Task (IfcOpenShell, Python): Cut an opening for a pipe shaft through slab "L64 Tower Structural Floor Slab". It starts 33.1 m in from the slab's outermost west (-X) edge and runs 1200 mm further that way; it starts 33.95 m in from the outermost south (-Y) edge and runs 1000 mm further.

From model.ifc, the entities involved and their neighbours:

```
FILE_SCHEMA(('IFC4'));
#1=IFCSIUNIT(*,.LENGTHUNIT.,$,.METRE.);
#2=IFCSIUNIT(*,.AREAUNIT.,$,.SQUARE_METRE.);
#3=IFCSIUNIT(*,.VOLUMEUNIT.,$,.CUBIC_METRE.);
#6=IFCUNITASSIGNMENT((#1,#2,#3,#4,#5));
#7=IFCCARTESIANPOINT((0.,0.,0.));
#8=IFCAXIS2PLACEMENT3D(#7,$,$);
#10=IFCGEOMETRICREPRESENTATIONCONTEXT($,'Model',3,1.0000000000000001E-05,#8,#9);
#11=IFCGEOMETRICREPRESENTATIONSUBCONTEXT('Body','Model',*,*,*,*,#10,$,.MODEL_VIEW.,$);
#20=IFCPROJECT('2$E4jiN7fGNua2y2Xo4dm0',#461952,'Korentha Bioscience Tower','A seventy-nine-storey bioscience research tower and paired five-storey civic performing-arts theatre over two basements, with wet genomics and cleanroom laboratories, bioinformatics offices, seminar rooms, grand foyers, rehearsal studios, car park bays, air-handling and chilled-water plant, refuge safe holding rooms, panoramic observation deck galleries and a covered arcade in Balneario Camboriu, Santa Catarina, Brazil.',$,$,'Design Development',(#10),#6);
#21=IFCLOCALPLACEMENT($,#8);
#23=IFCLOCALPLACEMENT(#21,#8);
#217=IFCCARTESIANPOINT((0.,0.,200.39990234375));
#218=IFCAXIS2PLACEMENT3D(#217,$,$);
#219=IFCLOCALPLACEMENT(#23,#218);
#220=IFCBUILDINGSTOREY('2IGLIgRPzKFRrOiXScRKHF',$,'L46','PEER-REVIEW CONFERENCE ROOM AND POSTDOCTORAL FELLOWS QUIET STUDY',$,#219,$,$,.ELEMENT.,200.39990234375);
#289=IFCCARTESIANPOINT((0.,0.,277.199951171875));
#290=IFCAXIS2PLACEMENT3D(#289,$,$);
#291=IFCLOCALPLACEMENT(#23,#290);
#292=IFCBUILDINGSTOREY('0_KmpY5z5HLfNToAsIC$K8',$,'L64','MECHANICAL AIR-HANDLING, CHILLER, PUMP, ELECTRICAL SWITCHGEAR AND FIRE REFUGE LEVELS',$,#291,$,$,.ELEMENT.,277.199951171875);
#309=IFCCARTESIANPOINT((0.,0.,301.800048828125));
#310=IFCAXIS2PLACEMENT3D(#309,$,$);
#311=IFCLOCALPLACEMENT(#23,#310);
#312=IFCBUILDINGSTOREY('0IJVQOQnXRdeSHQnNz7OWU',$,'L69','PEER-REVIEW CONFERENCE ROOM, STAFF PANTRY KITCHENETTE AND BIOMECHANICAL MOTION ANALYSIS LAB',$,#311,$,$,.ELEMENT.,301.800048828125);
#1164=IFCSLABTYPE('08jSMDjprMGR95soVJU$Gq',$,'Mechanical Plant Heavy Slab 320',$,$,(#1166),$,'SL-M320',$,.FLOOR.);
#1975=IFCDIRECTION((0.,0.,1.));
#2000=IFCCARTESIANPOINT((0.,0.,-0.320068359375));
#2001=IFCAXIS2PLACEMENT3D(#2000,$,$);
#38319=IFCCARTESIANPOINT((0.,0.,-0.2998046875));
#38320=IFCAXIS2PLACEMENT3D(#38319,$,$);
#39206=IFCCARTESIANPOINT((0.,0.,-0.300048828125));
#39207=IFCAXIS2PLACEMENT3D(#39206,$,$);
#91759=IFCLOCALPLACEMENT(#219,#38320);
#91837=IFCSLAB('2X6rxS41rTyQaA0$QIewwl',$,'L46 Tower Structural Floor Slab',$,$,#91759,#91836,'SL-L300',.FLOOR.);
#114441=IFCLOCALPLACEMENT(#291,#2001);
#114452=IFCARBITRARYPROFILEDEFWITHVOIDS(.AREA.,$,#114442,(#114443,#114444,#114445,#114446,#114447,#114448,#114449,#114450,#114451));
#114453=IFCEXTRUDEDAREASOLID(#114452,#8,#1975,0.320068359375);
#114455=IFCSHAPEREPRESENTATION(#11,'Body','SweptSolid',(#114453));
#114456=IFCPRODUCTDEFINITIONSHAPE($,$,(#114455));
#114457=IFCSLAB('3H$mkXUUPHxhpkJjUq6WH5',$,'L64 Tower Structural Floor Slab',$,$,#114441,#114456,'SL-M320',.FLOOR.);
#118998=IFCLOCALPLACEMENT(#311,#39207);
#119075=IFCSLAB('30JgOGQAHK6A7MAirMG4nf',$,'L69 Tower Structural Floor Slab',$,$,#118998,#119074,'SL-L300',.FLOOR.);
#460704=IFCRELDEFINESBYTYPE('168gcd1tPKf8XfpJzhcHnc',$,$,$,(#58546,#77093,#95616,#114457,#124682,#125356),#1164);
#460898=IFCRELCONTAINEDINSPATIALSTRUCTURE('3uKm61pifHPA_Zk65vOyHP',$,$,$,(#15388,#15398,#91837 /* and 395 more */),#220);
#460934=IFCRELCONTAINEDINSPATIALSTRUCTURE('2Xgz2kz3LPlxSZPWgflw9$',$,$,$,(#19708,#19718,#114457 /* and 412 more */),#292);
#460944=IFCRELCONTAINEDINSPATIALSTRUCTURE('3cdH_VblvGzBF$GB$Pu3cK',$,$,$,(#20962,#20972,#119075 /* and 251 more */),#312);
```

```python
import numpy as np
import ifcopenshell
import ifcopenshell.api.feature
import ifcopenshell.api.geometry
import ifcopenshell.api.root
import ifcopenshell.geom
import ifcopenshell.util.placement
import ifcopenshell.util.representation
import ifcopenshell.util.shape
import ifcopenshell.util.unit

model = ifcopenshell.open("model.ifc")
unit_scale = ifcopenshell.util.unit.calculate_unit_scale(model)
settings = ifcopenshell.geom.settings()


def volume(element):
    """Net volume in cubic metres, openings subtracted."""
    shape = ifcopenshell.geom.create_shape(settings, element)
    return ifcopenshell.util.shape.get_volume(shape.geometry)


slab = model.by_id(114457)
before = volume(slab)

# Extent in the slab's own axes, in metres. The edges named are its -X and -Y sides.
slab_shape = ifcopenshell.geom.create_shape(settings, slab)
vertices = ifcopenshell.util.shape.get_vertices(slab_shape.geometry)
x_min, y_min, bottom = vertices.min(axis=0)
top = vertices[:, 2].max()

opening = ifcopenshell.api.root.create_entity(model, ifc_class="IfcOpeningElement", name="Pipe shaft opening", predefined_type="OPENING")
context = ifcopenshell.util.representation.get_context(model, "Model", "Body", "MODEL_VIEW")
width, depth = 1.2, 1
outline = [(0.0, 0.0), (width, 0.0), (width, depth), (0.0, depth), (0.0, 0.0)]
# Overshoot both faces by 50 mm so the cut is clean.
shape = ifcopenshell.api.geometry.add_slab_representation(
    model, context=context, depth=top - bottom + 0.1, polyline=outline
)
ifcopenshell.api.geometry.assign_representation(model, product=opening, representation=shape)

matrix = ifcopenshell.util.placement.get_local_placement(slab.ObjectPlacement)
matrix[:, 3] = matrix @ np.append(np.array([x_min + 33.1, y_min + 33.95, bottom - 0.05]) / unit_scale, 1.0)
ifcopenshell.api.geometry.edit_object_placement(model, product=opening, matrix=matrix, is_si=False)
ifcopenshell.api.feature.add_feature(model, feature=opening, element=slab)

after = volume(slab)

print(f"slab volume {before:.3f} -> {after:.3f} m3")

model.write("model_rev.ifc")
```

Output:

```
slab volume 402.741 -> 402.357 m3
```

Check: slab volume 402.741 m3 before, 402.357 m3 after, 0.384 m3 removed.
